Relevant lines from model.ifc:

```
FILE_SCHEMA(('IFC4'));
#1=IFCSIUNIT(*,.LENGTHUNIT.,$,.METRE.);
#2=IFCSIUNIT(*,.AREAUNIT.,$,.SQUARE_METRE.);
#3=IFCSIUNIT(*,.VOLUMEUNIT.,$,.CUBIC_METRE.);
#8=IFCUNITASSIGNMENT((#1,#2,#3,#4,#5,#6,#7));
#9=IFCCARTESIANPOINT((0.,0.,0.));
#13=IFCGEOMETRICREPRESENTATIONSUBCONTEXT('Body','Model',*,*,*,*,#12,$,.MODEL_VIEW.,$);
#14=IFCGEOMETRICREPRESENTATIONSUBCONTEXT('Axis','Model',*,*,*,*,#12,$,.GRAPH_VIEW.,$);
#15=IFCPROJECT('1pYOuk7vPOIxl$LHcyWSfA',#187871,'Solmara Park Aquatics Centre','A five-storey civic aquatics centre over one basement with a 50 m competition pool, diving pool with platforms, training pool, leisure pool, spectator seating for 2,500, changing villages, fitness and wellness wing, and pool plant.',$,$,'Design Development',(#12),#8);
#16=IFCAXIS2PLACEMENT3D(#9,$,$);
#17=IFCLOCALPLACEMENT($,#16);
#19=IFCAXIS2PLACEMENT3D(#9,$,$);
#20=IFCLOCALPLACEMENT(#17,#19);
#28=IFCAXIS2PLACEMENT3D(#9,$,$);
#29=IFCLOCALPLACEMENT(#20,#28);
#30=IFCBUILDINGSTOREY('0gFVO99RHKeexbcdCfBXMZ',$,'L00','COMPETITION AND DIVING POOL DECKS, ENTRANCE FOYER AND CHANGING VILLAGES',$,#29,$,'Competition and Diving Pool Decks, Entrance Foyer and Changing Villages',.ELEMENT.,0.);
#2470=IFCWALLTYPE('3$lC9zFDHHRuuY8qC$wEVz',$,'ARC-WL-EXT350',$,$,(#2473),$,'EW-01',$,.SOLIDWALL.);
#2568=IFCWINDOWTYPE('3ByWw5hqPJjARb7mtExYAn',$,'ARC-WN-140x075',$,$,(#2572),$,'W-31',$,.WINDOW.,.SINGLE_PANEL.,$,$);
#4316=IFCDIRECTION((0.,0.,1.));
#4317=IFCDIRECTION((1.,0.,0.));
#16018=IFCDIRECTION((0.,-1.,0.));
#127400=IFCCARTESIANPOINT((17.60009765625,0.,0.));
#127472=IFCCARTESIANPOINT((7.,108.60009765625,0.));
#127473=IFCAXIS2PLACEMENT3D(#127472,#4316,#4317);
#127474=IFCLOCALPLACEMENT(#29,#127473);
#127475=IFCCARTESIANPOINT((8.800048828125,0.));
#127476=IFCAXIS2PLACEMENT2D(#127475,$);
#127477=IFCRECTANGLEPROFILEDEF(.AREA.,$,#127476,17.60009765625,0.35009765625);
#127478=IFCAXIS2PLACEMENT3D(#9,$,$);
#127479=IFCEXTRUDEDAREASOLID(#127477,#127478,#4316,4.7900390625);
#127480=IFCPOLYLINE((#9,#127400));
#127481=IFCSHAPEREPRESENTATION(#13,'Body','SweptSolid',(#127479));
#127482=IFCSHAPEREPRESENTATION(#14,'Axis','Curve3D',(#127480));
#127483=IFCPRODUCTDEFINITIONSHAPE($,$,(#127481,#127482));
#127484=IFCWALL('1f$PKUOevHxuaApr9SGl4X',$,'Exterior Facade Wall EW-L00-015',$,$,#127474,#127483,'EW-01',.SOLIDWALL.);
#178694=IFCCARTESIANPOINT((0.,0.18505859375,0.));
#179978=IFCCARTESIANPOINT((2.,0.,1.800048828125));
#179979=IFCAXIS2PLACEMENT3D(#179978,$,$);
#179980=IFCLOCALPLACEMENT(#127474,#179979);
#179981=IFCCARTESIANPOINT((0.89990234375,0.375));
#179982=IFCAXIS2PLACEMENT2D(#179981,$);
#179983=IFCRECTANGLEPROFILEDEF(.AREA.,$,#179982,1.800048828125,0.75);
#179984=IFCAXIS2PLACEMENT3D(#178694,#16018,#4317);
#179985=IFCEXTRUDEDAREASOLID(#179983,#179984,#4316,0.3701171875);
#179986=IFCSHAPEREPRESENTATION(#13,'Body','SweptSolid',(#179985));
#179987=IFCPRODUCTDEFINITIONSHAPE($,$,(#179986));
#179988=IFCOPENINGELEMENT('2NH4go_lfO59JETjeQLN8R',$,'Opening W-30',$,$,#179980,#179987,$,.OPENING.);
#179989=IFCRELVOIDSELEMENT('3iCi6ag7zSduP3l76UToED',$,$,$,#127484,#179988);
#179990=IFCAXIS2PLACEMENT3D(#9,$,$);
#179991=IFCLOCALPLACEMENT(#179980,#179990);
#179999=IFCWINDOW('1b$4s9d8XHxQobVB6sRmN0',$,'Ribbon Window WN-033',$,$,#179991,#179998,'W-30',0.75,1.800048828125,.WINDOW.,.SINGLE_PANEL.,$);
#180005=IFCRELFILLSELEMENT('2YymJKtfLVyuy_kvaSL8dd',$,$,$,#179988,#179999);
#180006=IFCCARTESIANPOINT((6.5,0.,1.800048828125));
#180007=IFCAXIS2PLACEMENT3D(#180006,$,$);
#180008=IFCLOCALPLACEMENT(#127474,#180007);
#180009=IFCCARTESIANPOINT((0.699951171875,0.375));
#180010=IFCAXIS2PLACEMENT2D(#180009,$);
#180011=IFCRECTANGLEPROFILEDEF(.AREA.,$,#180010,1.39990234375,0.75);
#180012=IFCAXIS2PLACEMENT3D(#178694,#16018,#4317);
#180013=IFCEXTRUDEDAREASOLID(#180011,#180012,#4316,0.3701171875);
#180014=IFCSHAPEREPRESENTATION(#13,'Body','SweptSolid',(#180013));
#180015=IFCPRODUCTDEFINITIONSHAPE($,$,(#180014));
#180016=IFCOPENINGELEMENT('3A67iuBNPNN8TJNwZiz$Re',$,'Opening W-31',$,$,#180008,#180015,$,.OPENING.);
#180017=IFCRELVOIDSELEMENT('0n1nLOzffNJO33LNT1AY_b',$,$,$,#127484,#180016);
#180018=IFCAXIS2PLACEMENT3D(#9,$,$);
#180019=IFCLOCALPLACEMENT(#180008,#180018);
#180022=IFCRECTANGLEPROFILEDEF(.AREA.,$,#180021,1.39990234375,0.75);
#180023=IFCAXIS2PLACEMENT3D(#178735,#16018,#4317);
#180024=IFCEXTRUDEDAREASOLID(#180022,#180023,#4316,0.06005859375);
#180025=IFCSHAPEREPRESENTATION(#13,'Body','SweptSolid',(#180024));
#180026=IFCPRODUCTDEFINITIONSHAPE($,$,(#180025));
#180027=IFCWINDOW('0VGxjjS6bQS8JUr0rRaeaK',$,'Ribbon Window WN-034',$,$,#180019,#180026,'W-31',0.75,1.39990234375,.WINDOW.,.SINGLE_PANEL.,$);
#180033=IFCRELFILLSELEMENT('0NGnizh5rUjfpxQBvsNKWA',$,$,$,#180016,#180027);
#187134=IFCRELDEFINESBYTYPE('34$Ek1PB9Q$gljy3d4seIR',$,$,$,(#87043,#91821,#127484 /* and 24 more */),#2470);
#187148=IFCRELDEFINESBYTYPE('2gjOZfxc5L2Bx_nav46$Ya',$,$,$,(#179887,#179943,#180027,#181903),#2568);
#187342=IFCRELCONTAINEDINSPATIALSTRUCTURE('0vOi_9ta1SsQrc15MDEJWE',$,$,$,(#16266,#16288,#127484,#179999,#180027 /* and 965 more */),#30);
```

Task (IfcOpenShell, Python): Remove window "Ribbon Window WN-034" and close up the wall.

```python
import ifcopenshell
import ifcopenshell.api.feature
import ifcopenshell.api.root
import ifcopenshell.geom
import ifcopenshell.util.shape

model = ifcopenshell.open("model.ifc")
settings = ifcopenshell.geom.settings()


def volume(element):
    """Net volume in cubic metres, openings subtracted."""
    shape = ifcopenshell.geom.create_shape(settings, element)
    return ifcopenshell.util.shape.get_volume(shape.geometry)


window = model.by_id(180027)
opening = window.FillsVoids[0].RelatingOpeningElement
wall = opening.VoidsElements[0].RelatingBuildingElement
before = volume(wall)

ifcopenshell.api.root.remove_product(model, product=window)
ifcopenshell.api.feature.remove_feature(model, feature=opening)

after = volume(wall)

print(f"wall volume {before:.3f} -> {after:.3f} m3")

model.write("model_v2.ifc")
```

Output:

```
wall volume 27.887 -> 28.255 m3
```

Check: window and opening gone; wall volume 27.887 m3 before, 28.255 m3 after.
